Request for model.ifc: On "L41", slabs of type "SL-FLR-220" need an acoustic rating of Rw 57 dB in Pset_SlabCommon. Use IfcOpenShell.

First a look at what the model holds.

```python
import ifcopenshell
import ifcopenshell.util.element

model = ifcopenshell.open("model.ifc")
print(model.schema)
storey = next(s for s in model.by_type("IfcBuildingStorey") if s.Name == "L41")
slabs = [e for e in ifcopenshell.util.element.get_decomposition(storey) if e.is_a("IfcSlab")]
seen = {}
for e in slabs:
    element_type = ifcopenshell.util.element.get_type(e)
    key = (element_type.Name if element_type != e and element_type else None, ifcopenshell.util.element.get_pset(e, "Pset_SlabCommon", "AcousticRating"))
    seen[key] = seen.get(key, 0) + 1
for (name, value), count in sorted(seen.items(), key=str):
    print(count, "x", name, "|", value)
```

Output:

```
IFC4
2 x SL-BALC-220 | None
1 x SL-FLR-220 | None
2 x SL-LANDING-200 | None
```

```python
import ifcopenshell
import ifcopenshell.api.pset
import ifcopenshell.util.element

model = ifcopenshell.open("model.ifc")

storey = next(s for s in model.by_type("IfcBuildingStorey") if s.Name == "L41")
slabs = [e for e in ifcopenshell.util.element.get_decomposition(storey) if e.is_a("IfcSlab")]

count = 0
for e in slabs:
    element_type = ifcopenshell.util.element.get_type(e)
    if element_type in (None, e) or element_type.Name != "SL-FLR-220":
        continue
    # add_pset returns the element's existing set when there is one.
    pset = ifcopenshell.api.pset.add_pset(model, product=e, name="Pset_SlabCommon")
    ifcopenshell.api.pset.edit_pset(model, pset=pset, properties={"AcousticRating": "Rw 57 dB"})
    count += 1

print(count, "slabs updated")

model.write("model_v2.ifc")
```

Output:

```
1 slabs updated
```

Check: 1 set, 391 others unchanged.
